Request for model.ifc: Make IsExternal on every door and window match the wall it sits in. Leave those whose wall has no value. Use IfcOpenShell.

First a look at what the model holds.

```python
import ifcopenshell
import ifcopenshell.util.element

model = ifcopenshell.open("model.ifc")
print(model.schema)
seen = {}
for e in model.by_type("IfcDoor") + model.by_type("IfcWindow"):
    if not e.FillsVoids:
        continue
    host = e.FillsVoids[0].RelatingOpeningElement.VoidsElements[0].RelatingBuildingElement
    own = ifcopenshell.util.element.get_pset(e, f"Pset_{e.is_a()[3:].removesuffix('StandardCase')}Common", "IsExternal")
    wall = ifcopenshell.util.element.get_pset(host, "Pset_WallCommon", "IsExternal")
    seen[e.is_a(), own, wall] = seen.get((e.is_a(), own, wall), 0) + 1
for (cls, own, wall), count in sorted(seen.items(), key=str):
    print(count, cls, "IsExternal:", own, "| host wall:", wall)
```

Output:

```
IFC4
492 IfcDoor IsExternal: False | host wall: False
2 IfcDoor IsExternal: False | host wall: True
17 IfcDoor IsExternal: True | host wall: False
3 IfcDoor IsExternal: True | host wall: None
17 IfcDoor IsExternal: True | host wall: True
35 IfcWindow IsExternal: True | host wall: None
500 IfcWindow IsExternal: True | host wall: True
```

```python
import ifcopenshell
import ifcopenshell.api.pset
import ifcopenshell.util.element

model = ifcopenshell.open("model.ifc")

count = 0
for ifc_class, pset_name in (("IfcDoor", "Pset_DoorCommon"), ("IfcWindow", "Pset_WindowCommon")):
    for e in model.by_type(ifc_class):
        if not e.FillsVoids:
            continue
        host = e.FillsVoids[0].RelatingOpeningElement.VoidsElements[0].RelatingBuildingElement
        external = ifcopenshell.util.element.get_pset(host, "Pset_WallCommon", "IsExternal")
        if external is None or ifcopenshell.util.element.get_pset(e, pset_name, "IsExternal") == external:
            continue
        pset = ifcopenshell.api.pset.add_pset(model, product=e, name=pset_name)
        ifcopenshell.api.pset.edit_pset(model, pset=pset, properties={"IsExternal": external})
        count += 1

print(count, "updated")

model.write("model-out.ifc")
```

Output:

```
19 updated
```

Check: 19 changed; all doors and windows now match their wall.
